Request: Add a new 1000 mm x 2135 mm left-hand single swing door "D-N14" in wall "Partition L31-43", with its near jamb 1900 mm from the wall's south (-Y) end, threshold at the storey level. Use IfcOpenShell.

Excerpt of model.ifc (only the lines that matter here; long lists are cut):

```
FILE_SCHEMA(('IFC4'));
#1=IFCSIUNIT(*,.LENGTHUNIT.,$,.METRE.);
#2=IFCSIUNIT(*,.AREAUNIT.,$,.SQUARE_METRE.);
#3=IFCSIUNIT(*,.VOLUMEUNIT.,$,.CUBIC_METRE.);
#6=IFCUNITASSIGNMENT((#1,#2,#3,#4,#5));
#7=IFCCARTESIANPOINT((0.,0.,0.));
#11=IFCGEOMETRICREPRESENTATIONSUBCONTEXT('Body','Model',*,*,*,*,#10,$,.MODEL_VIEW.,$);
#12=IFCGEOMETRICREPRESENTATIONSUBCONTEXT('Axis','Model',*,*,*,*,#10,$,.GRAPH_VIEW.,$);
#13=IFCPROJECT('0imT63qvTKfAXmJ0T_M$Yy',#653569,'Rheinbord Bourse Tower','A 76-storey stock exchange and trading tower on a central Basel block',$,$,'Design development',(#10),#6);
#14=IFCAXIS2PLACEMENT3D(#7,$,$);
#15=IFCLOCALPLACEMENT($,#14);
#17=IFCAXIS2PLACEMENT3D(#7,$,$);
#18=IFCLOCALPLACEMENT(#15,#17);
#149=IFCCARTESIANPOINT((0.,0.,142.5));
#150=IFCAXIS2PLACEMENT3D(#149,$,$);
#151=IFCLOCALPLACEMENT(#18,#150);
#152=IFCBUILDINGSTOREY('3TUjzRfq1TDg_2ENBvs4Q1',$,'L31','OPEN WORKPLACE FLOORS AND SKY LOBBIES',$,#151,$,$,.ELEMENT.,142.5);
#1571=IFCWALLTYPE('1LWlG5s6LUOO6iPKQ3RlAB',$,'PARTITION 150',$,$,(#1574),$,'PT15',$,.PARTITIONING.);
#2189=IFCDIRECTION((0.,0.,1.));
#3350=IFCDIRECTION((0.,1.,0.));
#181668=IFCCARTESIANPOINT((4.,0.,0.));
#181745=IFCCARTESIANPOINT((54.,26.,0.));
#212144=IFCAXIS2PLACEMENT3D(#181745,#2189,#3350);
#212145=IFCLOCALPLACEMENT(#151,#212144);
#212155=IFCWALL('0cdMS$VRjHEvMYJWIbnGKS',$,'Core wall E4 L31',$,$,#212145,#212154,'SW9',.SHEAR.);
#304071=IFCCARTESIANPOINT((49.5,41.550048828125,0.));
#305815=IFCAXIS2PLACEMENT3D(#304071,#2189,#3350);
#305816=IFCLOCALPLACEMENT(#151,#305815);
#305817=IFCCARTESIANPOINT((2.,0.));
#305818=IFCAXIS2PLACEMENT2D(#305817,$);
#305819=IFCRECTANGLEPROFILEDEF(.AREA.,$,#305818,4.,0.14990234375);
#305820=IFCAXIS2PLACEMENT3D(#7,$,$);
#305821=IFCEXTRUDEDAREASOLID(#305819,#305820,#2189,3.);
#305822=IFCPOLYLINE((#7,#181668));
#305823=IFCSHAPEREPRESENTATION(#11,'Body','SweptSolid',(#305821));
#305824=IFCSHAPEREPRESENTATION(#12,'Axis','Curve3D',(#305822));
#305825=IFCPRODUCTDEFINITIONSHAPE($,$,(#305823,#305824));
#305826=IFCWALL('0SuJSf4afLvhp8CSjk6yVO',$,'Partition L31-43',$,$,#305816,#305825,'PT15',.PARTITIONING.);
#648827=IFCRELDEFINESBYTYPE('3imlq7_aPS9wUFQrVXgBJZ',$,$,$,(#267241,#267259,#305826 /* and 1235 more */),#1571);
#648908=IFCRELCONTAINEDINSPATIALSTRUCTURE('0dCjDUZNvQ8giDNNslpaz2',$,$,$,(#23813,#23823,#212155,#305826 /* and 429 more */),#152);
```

```python
import numpy as np
import ifcopenshell
import ifcopenshell.api.feature
import ifcopenshell.api.geometry
import ifcopenshell.api.root
import ifcopenshell.api.spatial
import ifcopenshell.geom
import ifcopenshell.util.element
import ifcopenshell.util.placement
import ifcopenshell.util.representation
import ifcopenshell.util.shape
import ifcopenshell.util.unit

model = ifcopenshell.open("model.ifc")
unit_scale = ifcopenshell.util.unit.calculate_unit_scale(model)
settings = ifcopenshell.geom.settings()


def volume(element):
    """Net volume in cubic metres, openings subtracted."""
    shape = ifcopenshell.geom.create_shape(settings, element)
    return ifcopenshell.util.shape.get_volume(shape.geometry)


wall = model.by_guid("0SuJSf4afLvhp8CSjk6yVO")
storey = ifcopenshell.util.element.get_container(wall, ifc_class="IfcBuildingStorey")
context = ifcopenshell.util.representation.get_context(model, "Model", "Body", "MODEL_VIEW")
before = volume(wall)

width, height, from_end, sill = 1, 2.135, 1.9, 0.0  # metres

# The wall runs along its own X axis, and the end named is its -X end.
wall_shape = ifcopenshell.geom.create_shape(settings, wall)
x, y, z = ifcopenshell.util.shape.get_vertices(wall_shape.geometry).T
start = x.min() + from_end
face, thickness = float(y.min()), float(y.max() - y.min())
wall_matrix = ifcopenshell.util.placement.get_local_placement(wall.ObjectPlacement)
level = ifcopenshell.util.placement.get_local_placement(storey.ObjectPlacement)[2, 3]


def in_wall(x, y):
    """Placement at x, y metres in the wall's axes, at sill height."""
    matrix = wall_matrix.copy()
    matrix[:, 3] = wall_matrix @ np.array([x / unit_scale, y / unit_scale, 0.0, 1.0])
    matrix[2, 3] = level + sill / unit_scale
    return matrix


# Opening: a box that overshoots both wall faces by 50 mm.
opening = ifcopenshell.api.root.create_entity(model, ifc_class="IfcOpeningElement", predefined_type="OPENING")
box = ifcopenshell.api.geometry.add_wall_representation(
    model, context=context, length=width, height=height, thickness=thickness + 0.1
)
ifcopenshell.api.geometry.assign_representation(model, product=opening, representation=box)
ifcopenshell.api.geometry.edit_object_placement(model, product=opening, matrix=in_wall(start, face - 0.05), is_si=False)
ifcopenshell.api.feature.add_feature(model, feature=opening, element=wall)

door = ifcopenshell.api.root.create_entity(model, ifc_class="IfcDoor", name="D-N14", predefined_type="DOOR")
door.OverallWidth, door.OverallHeight = width / unit_scale, height / unit_scale
door.OperationType = "SINGLE_SWING_LEFT"
body = ifcopenshell.api.geometry.add_door_representation(
    model,
    context=context,
    overall_width=door.OverallWidth,
    overall_height=door.OverallHeight,
    operation_type="SINGLE_SWING_LEFT",
    lining_properties={"LiningDepth": thickness / unit_scale, "ThresholdDepth": thickness / unit_scale},
)
ifcopenshell.api.geometry.assign_representation(model, product=door, representation=body)
ifcopenshell.api.spatial.assign_container(model, products=[door], relating_structure=storey)
ifcopenshell.api.feature.add_filling(model, opening=opening, element=door)

# The lining spans the wall, so the door starts at the wall face.
ifcopenshell.api.geometry.edit_object_placement(model, product=door, matrix=in_wall(start, face), is_si=False)

after = volume(wall)

print(f"wall volume {before:.3f} -> {after:.3f} m3")

model.write("model_rev.ifc")
```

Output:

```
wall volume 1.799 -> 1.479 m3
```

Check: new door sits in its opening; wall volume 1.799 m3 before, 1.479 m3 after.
